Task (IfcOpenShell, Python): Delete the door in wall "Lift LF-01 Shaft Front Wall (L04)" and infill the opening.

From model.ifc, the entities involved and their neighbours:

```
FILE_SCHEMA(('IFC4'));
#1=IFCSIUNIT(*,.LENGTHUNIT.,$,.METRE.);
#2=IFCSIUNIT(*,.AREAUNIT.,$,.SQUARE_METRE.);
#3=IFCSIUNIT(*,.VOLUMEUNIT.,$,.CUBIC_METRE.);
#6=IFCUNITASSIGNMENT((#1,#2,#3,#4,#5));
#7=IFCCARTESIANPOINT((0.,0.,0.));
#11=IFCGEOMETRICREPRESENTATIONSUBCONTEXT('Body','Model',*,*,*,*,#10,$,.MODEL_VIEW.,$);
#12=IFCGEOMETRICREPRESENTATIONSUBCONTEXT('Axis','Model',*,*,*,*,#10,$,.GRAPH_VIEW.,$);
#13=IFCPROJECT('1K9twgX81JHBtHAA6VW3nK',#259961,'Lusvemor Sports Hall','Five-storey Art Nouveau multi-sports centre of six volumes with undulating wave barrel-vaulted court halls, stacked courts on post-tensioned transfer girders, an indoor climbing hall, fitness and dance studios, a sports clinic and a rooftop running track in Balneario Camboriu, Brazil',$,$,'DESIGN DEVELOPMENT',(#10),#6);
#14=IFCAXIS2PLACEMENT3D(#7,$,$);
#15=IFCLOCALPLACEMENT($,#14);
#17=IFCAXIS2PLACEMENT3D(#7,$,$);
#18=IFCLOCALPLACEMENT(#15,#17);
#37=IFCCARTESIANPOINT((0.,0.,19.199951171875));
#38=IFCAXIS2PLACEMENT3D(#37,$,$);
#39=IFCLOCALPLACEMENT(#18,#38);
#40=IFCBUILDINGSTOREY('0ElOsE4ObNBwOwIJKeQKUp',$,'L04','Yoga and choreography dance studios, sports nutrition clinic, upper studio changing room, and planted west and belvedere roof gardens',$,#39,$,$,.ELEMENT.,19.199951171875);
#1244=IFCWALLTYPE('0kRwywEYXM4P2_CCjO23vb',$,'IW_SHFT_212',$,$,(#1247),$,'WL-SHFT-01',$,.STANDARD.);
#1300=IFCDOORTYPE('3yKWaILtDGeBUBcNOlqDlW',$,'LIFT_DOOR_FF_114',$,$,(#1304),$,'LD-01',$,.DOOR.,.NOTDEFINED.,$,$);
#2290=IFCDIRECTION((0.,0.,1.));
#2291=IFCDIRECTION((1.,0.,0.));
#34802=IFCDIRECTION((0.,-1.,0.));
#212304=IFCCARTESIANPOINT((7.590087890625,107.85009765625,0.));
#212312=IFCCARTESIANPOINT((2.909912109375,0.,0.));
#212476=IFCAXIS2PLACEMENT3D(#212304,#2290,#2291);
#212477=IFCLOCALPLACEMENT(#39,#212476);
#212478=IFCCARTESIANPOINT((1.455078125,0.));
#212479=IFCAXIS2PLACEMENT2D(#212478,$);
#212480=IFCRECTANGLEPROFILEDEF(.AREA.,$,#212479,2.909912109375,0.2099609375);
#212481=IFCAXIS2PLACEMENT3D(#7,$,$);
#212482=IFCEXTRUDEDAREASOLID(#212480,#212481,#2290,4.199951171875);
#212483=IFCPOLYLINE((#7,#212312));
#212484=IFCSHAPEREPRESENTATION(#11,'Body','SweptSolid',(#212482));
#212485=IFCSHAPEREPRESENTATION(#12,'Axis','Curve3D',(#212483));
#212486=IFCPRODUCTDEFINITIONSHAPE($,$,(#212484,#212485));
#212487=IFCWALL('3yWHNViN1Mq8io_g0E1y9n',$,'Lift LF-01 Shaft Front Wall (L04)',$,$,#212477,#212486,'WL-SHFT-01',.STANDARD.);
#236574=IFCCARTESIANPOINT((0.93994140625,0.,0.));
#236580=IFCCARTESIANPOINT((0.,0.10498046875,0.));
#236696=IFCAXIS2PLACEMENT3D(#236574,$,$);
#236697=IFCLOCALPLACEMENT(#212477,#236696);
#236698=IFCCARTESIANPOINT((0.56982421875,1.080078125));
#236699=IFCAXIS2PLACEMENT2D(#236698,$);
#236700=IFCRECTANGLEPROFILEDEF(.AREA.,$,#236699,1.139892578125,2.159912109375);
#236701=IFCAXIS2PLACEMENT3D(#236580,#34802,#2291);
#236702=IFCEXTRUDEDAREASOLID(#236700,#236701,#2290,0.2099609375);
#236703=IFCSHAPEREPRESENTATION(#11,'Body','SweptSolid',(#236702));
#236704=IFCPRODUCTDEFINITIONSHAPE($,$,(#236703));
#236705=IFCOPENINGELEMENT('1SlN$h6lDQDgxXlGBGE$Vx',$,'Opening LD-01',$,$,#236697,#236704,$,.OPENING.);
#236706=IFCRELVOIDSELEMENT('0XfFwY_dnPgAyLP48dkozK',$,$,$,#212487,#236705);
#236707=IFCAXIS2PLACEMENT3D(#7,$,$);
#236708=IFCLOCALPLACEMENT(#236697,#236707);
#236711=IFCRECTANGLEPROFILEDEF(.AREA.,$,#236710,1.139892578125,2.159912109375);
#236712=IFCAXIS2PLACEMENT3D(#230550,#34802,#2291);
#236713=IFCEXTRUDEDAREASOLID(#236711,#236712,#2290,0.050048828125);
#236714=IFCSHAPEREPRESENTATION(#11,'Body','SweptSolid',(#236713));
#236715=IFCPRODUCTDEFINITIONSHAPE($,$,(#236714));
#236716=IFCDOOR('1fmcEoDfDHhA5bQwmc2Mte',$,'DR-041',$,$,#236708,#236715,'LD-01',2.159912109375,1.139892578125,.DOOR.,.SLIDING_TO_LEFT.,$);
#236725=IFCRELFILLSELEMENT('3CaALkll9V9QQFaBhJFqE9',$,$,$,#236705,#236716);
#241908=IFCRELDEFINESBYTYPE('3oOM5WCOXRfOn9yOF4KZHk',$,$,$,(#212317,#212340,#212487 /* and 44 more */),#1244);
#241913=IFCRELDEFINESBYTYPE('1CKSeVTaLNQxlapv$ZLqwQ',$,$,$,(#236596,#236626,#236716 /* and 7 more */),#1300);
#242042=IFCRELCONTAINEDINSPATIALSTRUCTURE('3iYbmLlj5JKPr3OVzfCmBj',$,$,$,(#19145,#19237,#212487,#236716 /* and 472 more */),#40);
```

```python
import ifcopenshell
import ifcopenshell.api.feature
import ifcopenshell.api.root
import ifcopenshell.geom
import ifcopenshell.util.shape

model = ifcopenshell.open("model.ifc")
settings = ifcopenshell.geom.settings()


def volume(element):
    """Net volume in cubic metres, openings subtracted."""
    shape = ifcopenshell.geom.create_shape(settings, element)
    return ifcopenshell.util.shape.get_volume(shape.geometry)


door = model.by_guid("1fmcEoDfDHhA5bQwmc2Mte")
opening = door.FillsVoids[0].RelatingOpeningElement
wall = opening.VoidsElements[0].RelatingBuildingElement
before = volume(wall)

ifcopenshell.api.root.remove_product(model, product=door)
ifcopenshell.api.feature.remove_feature(model, feature=opening)

after = volume(wall)

print(f"wall volume {before:.3f} -> {after:.3f} m3")

model.write("model_edited.ifc")
```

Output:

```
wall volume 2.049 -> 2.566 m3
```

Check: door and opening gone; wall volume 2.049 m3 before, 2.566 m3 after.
